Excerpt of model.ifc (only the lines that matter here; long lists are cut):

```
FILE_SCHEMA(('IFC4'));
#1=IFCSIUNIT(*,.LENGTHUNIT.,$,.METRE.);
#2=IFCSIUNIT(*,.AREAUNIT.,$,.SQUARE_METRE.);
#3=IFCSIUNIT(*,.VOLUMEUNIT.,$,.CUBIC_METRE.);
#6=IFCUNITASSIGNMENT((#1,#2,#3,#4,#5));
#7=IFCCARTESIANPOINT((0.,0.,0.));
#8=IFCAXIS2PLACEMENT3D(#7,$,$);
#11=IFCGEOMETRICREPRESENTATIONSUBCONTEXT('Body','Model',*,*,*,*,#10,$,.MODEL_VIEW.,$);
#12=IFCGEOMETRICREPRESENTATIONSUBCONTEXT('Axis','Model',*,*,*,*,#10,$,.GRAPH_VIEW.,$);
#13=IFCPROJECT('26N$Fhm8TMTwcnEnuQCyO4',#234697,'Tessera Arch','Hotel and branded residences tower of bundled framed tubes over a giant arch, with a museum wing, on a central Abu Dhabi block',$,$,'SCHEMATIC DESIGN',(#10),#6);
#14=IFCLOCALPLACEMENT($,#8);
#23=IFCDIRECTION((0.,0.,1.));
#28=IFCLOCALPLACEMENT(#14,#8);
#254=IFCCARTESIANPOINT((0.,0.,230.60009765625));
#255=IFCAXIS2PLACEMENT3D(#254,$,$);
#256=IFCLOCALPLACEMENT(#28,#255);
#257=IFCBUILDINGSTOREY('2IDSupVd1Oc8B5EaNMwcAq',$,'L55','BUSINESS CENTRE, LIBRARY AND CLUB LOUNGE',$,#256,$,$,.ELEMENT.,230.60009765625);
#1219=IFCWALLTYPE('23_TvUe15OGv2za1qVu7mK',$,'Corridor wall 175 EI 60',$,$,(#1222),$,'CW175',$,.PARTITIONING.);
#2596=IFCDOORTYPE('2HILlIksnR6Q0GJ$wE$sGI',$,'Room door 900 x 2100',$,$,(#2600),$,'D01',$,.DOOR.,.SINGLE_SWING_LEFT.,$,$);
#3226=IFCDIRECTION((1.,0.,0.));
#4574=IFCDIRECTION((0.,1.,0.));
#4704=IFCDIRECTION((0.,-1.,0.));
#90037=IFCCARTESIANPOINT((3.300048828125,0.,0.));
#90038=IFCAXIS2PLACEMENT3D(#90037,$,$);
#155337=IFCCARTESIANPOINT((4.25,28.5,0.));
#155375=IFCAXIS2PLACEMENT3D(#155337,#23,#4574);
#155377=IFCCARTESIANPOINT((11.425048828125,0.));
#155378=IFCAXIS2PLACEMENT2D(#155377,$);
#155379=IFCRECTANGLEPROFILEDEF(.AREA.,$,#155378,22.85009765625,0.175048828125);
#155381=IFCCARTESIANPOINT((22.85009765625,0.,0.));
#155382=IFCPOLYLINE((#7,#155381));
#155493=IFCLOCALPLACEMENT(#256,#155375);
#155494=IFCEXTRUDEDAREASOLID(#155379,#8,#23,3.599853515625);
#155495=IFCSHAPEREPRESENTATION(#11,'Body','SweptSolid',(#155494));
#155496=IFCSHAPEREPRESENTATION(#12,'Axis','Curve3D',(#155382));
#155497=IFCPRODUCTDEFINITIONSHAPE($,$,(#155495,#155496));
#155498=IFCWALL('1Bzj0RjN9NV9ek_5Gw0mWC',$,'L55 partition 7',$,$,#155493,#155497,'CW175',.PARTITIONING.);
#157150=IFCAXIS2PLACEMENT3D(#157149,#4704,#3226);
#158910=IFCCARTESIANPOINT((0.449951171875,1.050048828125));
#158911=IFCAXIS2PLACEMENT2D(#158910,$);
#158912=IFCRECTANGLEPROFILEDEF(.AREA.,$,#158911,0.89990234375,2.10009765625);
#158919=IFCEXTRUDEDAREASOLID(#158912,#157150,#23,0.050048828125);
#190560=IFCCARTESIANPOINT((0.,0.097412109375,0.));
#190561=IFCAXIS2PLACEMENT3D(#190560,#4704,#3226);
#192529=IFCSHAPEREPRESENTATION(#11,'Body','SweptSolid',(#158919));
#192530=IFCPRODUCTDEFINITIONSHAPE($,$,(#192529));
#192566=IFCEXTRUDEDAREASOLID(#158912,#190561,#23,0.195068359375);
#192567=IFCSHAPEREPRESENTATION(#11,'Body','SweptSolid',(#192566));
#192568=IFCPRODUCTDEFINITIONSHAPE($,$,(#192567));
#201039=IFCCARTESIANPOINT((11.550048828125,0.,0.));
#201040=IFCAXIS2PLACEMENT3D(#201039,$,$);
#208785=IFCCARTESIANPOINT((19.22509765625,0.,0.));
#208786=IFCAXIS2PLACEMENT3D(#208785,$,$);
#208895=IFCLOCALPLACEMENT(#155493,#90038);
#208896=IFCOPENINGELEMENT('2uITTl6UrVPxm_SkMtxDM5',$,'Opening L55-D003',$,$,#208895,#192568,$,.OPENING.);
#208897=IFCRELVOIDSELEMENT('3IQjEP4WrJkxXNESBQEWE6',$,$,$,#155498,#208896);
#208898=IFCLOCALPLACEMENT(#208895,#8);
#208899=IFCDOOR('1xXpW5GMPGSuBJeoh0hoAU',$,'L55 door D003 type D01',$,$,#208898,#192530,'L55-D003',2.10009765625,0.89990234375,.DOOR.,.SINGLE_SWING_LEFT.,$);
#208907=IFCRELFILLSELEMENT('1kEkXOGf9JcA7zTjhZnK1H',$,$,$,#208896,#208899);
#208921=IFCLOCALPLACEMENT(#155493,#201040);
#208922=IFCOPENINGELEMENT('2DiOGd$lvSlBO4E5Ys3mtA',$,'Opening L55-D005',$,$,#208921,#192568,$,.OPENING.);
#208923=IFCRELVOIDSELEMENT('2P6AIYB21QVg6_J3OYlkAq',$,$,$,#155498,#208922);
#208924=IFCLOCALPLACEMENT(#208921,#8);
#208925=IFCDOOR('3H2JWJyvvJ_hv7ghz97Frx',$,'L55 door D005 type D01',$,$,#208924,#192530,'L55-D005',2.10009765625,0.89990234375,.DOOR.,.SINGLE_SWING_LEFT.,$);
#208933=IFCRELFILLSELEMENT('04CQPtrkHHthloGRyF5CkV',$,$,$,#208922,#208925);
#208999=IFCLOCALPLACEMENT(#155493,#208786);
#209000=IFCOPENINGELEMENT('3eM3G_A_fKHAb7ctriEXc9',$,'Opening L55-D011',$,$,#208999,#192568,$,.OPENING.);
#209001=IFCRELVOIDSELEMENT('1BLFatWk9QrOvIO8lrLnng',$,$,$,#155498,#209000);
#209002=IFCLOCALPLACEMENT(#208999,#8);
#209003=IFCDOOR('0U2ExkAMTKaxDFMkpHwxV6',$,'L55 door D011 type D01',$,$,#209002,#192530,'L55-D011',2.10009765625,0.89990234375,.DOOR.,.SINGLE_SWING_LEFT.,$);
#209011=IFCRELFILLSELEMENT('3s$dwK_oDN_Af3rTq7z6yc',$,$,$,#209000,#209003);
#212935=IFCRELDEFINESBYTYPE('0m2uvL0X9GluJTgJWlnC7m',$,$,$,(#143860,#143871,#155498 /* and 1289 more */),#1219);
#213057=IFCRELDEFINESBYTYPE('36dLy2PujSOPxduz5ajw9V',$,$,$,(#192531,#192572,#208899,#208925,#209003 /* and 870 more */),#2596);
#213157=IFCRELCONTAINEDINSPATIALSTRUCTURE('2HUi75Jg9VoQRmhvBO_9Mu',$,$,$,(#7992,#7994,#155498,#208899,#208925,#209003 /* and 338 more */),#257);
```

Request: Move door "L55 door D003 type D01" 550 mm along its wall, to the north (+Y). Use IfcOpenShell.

```python
import ifcopenshell
import ifcopenshell.api.geometry
import ifcopenshell.util.placement
import ifcopenshell.util.unit

model = ifcopenshell.open("model.ifc")
unit_scale = ifcopenshell.util.unit.calculate_unit_scale(model)

door = model.by_guid("1xXpW5GMPGSuBJeoh0hoAU")
opening = door.FillsVoids[0].RelatingOpeningElement
wall = opening.VoidsElements[0].RelatingBuildingElement

wall_matrix = ifcopenshell.util.placement.get_local_placement(wall.ObjectPlacement)
shift = wall_matrix[:3, 0] * 0.55 / unit_scale
before = ifcopenshell.util.placement.get_local_placement(door.ObjectPlacement)[:3, 3].copy()

# The door is placed relative to its opening, so it follows when the opening moves.
matrix = ifcopenshell.util.placement.get_local_placement(opening.ObjectPlacement)
matrix[:3, 3] += shift
ifcopenshell.api.geometry.edit_object_placement(
    model, product=opening, matrix=matrix, is_si=False, should_transform_children=True
)

after = ifcopenshell.util.placement.get_local_placement(door.ObjectPlacement)[:3, 3]
print("door moved by", (after - before).round(3) + 0.0)

model.write("model_edited.ifc")
```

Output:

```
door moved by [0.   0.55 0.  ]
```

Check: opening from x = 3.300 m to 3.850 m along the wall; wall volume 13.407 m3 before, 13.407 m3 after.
